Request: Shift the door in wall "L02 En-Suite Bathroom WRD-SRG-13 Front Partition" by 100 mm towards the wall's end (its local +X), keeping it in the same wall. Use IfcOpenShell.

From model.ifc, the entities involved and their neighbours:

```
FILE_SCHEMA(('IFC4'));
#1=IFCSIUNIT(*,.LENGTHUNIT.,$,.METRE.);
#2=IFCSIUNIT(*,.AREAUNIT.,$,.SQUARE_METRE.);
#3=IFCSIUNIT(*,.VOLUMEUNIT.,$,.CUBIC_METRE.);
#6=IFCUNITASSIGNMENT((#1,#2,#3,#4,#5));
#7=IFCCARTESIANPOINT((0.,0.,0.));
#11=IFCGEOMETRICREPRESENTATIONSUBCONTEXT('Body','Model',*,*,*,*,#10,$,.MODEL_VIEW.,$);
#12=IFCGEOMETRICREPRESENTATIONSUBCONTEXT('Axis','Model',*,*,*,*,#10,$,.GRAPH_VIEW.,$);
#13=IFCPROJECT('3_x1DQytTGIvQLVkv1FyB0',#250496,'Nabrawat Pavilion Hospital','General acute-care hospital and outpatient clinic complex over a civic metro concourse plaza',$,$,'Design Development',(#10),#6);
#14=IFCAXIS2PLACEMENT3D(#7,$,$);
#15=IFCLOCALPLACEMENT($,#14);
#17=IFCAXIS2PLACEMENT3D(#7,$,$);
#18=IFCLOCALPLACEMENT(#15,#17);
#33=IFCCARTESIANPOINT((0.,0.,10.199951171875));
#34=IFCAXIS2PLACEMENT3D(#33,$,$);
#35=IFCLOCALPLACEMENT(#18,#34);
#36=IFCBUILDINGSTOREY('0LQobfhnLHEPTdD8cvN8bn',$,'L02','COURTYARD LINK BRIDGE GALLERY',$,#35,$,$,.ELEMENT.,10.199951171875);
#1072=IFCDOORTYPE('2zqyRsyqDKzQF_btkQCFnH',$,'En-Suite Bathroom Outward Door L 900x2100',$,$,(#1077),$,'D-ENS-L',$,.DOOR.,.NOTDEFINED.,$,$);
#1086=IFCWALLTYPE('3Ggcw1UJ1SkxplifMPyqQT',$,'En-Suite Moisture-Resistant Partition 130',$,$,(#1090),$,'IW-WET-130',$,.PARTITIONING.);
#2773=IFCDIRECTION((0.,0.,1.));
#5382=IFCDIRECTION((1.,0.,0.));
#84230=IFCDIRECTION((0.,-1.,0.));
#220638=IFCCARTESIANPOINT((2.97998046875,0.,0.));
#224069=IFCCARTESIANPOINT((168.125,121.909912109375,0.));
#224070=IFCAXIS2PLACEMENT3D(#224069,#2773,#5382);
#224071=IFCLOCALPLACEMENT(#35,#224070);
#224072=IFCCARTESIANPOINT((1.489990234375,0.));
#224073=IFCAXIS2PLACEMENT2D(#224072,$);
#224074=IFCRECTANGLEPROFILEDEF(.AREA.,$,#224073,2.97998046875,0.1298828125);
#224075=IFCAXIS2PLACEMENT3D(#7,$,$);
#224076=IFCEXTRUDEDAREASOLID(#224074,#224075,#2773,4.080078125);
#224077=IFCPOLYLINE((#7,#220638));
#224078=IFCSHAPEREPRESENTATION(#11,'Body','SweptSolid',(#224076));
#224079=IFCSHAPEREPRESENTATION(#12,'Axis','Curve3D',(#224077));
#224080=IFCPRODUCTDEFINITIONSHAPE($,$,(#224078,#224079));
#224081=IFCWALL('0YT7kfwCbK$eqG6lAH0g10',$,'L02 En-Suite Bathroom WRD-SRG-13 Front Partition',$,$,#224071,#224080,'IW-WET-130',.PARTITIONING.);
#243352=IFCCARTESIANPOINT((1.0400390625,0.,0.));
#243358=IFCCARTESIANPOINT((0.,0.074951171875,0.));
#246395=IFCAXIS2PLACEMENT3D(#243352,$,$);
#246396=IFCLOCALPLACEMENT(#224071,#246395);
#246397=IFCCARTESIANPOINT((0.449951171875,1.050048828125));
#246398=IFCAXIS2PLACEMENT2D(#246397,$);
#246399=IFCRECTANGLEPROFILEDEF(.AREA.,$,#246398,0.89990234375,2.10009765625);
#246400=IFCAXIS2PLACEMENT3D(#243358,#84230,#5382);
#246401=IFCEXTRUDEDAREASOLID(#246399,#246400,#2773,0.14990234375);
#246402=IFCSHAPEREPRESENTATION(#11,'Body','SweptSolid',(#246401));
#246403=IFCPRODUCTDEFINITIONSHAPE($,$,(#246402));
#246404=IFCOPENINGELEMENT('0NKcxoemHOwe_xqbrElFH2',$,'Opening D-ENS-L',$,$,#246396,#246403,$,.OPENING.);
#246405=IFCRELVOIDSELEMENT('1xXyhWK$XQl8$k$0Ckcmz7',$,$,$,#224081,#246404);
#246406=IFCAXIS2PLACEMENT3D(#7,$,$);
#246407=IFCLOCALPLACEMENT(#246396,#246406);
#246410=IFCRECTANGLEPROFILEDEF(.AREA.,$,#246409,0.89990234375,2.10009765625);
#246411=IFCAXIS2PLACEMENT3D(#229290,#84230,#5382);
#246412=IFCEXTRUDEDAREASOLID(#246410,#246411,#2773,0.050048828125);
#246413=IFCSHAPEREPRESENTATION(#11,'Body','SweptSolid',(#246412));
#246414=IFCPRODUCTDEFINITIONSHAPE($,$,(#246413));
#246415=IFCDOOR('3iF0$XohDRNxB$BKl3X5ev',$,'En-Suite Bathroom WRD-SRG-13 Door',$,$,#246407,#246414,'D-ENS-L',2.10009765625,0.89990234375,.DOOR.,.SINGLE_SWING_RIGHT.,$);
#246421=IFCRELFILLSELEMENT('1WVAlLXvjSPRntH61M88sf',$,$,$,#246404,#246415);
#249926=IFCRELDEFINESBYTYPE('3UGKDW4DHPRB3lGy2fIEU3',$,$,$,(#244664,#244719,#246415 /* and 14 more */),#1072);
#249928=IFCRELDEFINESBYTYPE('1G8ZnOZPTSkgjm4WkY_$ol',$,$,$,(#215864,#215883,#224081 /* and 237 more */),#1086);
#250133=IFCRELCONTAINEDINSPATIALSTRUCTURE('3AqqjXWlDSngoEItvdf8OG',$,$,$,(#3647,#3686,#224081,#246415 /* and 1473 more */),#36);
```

```python
import ifcopenshell
import ifcopenshell.api.geometry
import ifcopenshell.util.placement

model = ifcopenshell.open("model.ifc")

door = model.by_guid("3iF0$XohDRNxB$BKl3X5ev")
opening = door.FillsVoids[0].RelatingOpeningElement
wall = opening.VoidsElements[0].RelatingBuildingElement

wall_matrix = ifcopenshell.util.placement.get_local_placement(wall.ObjectPlacement)
shift = wall_matrix[:3, 0] * 0.1
before = ifcopenshell.util.placement.get_local_placement(door.ObjectPlacement)[:3, 3].copy()

# The door is placed relative to its opening, so it follows when the opening moves.
matrix = ifcopenshell.util.placement.get_local_placement(opening.ObjectPlacement)
matrix[:3, 3] += shift
ifcopenshell.api.geometry.edit_object_placement(
    model, product=opening, matrix=matrix, is_si=False, should_transform_children=True
)

after = ifcopenshell.util.placement.get_local_placement(door.ObjectPlacement)[:3, 3]
print("door moved by", (after - before).round(3) + 0.0)

model.write("model_rev.ifc")
```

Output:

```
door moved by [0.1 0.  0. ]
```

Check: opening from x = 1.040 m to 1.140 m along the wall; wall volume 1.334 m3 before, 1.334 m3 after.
